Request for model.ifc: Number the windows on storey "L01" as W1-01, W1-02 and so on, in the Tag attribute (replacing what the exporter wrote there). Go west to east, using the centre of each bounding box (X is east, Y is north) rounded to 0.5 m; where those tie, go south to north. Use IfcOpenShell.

First a look at what the model holds.

```python
import ifcopenshell
import ifcopenshell.util.element
import ifcopenshell.util.placement

model = ifcopenshell.open("model.ifc")
print(model.schema)
storey = next(s for s in model.by_type("IfcBuildingStorey") if s.Name == "L01")
windows = [e for e in ifcopenshell.util.element.get_decomposition(storey) if e.is_a("IfcWindow")]
for e in sorted(windows, key=lambda e: e.id()):
    origin = ifcopenshell.util.placement.get_local_placement(e.ObjectPlacement)[:3, 3]
    print(e.id(), e.Tag, e.Name, origin.round(2) + 0.0, sep=" | ")
```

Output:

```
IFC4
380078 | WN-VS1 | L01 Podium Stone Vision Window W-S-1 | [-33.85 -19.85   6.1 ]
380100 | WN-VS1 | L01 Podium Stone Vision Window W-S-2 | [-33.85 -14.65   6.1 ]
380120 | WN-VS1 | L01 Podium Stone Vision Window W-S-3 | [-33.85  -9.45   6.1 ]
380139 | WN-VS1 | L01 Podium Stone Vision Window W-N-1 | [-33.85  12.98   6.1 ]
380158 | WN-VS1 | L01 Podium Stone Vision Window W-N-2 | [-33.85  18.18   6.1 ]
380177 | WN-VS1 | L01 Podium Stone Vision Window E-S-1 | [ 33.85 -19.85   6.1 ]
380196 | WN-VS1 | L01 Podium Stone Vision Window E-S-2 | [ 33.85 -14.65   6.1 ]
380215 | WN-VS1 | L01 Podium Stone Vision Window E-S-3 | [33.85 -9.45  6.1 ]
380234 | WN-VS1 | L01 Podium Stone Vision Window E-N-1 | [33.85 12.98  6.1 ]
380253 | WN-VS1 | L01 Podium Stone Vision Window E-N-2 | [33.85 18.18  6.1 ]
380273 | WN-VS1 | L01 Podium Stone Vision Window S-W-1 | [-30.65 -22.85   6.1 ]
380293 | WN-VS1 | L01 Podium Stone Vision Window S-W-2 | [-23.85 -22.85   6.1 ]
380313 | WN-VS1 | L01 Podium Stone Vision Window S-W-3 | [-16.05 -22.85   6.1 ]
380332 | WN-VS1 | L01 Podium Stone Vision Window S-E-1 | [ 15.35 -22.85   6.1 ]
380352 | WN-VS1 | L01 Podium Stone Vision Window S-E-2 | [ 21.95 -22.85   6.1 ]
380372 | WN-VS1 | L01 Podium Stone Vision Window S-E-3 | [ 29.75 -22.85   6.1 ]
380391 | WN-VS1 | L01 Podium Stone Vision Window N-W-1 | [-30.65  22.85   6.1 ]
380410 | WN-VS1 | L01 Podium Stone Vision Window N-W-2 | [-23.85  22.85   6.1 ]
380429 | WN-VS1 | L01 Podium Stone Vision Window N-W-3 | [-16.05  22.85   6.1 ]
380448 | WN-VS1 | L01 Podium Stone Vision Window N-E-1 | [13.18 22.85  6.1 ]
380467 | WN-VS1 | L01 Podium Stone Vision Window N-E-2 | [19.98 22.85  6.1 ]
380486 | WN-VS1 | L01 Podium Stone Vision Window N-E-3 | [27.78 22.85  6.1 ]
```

```python
import ifcopenshell
import ifcopenshell.geom
import ifcopenshell.util.element
import ifcopenshell.util.shape

model = ifcopenshell.open("model.ifc")
settings = ifcopenshell.geom.settings()
settings.set("use-world-coords", True)


def centre(element):
    shape = ifcopenshell.geom.create_shape(settings, element)
    return ifcopenshell.util.shape.get_bbox_centroid(shape.geometry)


storey = next(s for s in model.by_type("IfcBuildingStorey") if s.Name == "L01")
windows = [e for e in ifcopenshell.util.element.get_decomposition(storey) if e.is_a("IfcWindow")]

# Insertion points can sit at a corner or the storey origin, so sort by the geometry (in metres).
centres = {e: centre(e) for e in windows}
windows.sort(key=lambda e: (round(centres[e][0] / 0.5), centres[e][1]))

for i, e in enumerate(windows, start=1):
    number = f"W1-{i:02d}"
    e.Tag = number
    print(e.id(), number)

model.write("model-out.ifc")
```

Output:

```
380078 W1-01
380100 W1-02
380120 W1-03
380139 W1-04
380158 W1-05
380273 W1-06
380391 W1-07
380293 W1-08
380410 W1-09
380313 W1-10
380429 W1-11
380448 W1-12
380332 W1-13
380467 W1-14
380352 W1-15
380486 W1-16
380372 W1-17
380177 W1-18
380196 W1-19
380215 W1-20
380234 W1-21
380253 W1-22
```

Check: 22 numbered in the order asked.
